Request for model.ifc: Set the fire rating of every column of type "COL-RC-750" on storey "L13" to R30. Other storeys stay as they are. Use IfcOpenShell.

First a look at what the model holds.

```python
import ifcopenshell
import ifcopenshell.util.element

model = ifcopenshell.open("model.ifc")
print(model.schema)
storey = next(s for s in model.by_type("IfcBuildingStorey") if s.Name == "L13")
columns = [e for e in ifcopenshell.util.element.get_decomposition(storey) if e.is_a("IfcColumn")]
seen = {}
for e in columns:
    element_type = ifcopenshell.util.element.get_type(e)
    key = (element_type.Name if element_type != e and element_type else None, ifcopenshell.util.element.get_pset(e, "Pset_ColumnCommon", "FireRating"))
    seen[key] = seen.get(key, 0) + 1
for (name, value), count in sorted(seen.items(), key=str):
    print(count, "x", name, "|", value)
```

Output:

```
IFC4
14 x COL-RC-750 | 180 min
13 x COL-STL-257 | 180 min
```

```python
import ifcopenshell
import ifcopenshell.api.pset
import ifcopenshell.util.element

model = ifcopenshell.open("model.ifc")

storey = next(s for s in model.by_type("IfcBuildingStorey") if s.Name == "L13")
columns = [e for e in ifcopenshell.util.element.get_decomposition(storey) if e.is_a("IfcColumn")]

count = 0
for e in columns:
    element_type = ifcopenshell.util.element.get_type(e)
    if element_type in (None, e) or element_type.Name != "COL-RC-750":
        continue
    # add_pset returns the element's existing set when there is one.
    pset = ifcopenshell.api.pset.add_pset(model, product=e, name="Pset_ColumnCommon")
    ifcopenshell.api.pset.edit_pset(model, pset=pset, properties={"FireRating": "R30"})
    count += 1

print(count, "columns updated")

model.write("model_edited.ifc")
```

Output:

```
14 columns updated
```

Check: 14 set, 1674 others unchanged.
